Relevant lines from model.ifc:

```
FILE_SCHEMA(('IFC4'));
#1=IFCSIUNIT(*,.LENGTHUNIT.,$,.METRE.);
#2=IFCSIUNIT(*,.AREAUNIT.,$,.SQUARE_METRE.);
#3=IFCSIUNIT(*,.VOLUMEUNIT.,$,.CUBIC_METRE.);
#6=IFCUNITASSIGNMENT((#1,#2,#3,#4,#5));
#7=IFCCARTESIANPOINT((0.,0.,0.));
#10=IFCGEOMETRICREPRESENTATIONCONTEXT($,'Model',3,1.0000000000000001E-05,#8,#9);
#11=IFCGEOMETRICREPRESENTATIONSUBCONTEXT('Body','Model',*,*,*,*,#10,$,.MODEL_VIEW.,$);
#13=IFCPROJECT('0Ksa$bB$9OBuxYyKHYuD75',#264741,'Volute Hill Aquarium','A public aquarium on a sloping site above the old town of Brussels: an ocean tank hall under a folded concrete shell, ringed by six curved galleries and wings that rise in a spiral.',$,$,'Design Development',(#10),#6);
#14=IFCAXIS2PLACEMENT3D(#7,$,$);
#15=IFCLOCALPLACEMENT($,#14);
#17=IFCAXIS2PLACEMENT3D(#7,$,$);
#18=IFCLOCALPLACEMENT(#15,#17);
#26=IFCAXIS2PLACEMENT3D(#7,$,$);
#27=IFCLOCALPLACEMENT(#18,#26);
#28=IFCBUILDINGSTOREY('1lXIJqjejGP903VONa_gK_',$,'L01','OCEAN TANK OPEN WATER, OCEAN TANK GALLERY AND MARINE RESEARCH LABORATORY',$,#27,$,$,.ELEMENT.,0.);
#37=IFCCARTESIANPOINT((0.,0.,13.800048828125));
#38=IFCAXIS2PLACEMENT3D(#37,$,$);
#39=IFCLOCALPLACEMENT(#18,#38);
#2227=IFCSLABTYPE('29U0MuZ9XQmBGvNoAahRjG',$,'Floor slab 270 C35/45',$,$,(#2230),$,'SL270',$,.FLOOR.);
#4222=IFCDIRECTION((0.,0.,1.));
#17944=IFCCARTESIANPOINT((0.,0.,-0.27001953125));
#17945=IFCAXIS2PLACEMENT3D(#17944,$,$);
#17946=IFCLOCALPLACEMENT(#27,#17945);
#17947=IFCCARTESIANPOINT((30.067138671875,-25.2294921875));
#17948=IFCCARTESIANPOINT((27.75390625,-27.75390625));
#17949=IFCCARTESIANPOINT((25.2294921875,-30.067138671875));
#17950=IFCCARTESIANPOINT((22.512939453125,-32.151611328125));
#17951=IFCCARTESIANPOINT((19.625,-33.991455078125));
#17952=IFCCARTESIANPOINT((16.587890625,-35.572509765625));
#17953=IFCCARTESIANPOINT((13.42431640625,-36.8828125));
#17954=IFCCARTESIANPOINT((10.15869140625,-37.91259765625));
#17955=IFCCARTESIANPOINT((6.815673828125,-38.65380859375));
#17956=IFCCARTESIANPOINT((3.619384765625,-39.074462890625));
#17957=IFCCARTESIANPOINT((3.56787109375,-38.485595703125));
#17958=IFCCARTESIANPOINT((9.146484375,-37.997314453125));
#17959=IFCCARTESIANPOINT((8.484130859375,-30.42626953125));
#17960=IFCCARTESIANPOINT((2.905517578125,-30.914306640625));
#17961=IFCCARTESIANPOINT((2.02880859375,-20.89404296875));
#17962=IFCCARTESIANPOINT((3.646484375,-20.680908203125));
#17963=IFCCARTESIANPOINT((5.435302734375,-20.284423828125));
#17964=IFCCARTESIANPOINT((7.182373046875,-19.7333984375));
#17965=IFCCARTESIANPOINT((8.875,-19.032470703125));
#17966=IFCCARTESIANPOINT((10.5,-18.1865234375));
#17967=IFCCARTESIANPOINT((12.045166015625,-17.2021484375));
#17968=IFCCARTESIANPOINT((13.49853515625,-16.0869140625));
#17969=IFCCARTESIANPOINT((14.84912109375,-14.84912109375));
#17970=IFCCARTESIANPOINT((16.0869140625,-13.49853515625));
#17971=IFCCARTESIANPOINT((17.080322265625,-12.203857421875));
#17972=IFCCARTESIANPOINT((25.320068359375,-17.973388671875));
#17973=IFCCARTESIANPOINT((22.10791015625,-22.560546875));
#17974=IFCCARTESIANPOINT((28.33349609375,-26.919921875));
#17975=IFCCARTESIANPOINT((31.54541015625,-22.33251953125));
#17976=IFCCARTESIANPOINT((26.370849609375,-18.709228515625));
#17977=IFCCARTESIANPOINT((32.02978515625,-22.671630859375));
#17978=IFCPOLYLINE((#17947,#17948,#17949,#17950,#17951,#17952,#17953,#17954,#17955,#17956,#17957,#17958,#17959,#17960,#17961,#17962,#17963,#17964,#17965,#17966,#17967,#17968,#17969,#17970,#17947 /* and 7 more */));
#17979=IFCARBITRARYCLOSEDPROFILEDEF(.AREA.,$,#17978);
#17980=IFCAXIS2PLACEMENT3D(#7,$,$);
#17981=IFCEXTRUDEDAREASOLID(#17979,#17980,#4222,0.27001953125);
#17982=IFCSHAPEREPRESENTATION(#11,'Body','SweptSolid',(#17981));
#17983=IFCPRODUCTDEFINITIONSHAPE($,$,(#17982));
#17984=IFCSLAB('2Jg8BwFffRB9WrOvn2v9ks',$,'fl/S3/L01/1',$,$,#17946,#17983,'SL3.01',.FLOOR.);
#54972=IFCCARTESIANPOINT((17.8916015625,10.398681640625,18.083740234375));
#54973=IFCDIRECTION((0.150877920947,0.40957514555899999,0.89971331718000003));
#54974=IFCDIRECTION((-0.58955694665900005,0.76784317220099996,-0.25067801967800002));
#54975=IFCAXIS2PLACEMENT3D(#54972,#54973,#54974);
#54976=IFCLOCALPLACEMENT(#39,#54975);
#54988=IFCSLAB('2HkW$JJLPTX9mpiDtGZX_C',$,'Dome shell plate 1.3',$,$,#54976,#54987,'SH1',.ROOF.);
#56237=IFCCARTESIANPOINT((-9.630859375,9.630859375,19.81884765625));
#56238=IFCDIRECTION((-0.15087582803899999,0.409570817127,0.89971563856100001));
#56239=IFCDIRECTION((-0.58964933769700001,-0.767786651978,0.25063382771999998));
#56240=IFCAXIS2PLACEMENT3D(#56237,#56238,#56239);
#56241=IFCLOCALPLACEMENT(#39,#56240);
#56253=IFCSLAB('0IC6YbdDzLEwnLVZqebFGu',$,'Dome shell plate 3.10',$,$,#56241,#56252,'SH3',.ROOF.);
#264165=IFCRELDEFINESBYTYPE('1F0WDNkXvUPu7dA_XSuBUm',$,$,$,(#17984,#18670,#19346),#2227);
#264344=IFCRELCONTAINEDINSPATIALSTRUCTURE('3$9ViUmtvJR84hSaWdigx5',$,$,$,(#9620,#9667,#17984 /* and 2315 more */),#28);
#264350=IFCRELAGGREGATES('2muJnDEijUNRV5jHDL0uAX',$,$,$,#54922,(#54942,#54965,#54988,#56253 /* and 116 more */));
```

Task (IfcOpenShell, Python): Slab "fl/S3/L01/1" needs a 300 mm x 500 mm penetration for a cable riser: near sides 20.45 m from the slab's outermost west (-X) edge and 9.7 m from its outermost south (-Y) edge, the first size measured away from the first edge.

```python
import numpy as np
import ifcopenshell
import ifcopenshell.api.feature
import ifcopenshell.api.geometry
import ifcopenshell.api.root
import ifcopenshell.geom
import ifcopenshell.util.placement
import ifcopenshell.util.representation
import ifcopenshell.util.shape
import ifcopenshell.util.unit

model = ifcopenshell.open("model.ifc")
unit_scale = ifcopenshell.util.unit.calculate_unit_scale(model)
settings = ifcopenshell.geom.settings()


def volume(element):
    """Net volume in cubic metres, openings subtracted."""
    shape = ifcopenshell.geom.create_shape(settings, element)
    return ifcopenshell.util.shape.get_volume(shape.geometry)


slab = model.by_guid("2Jg8BwFffRB9WrOvn2v9ks")
before = volume(slab)

# Extent in the slab's own axes, in metres. The edges named are its -X and -Y sides.
slab_shape = ifcopenshell.geom.create_shape(settings, slab)
vertices = ifcopenshell.util.shape.get_vertices(slab_shape.geometry)
x_min, y_min, bottom = vertices.min(axis=0)
top = vertices[:, 2].max()

opening = ifcopenshell.api.root.create_entity(model, ifc_class="IfcOpeningElement", name="Cable riser opening", predefined_type="OPENING")
context = ifcopenshell.util.representation.get_context(model, "Model", "Body", "MODEL_VIEW")
width, depth = 0.3, 0.5
outline = [(0.0, 0.0), (width, 0.0), (width, depth), (0.0, depth), (0.0, 0.0)]
# Overshoot both faces by 50 mm so the cut is clean.
shape = ifcopenshell.api.geometry.add_slab_representation(
    model, context=context, depth=top - bottom + 0.1, polyline=outline
)
ifcopenshell.api.geometry.assign_representation(model, product=opening, representation=shape)

matrix = ifcopenshell.util.placement.get_local_placement(slab.ObjectPlacement)
matrix[:, 3] = matrix @ np.append(np.array([x_min + 20.45, y_min + 9.7, bottom - 0.05]) / unit_scale, 1.0)
ifcopenshell.api.geometry.edit_object_placement(model, product=opening, matrix=matrix, is_si=False)
ifcopenshell.api.feature.add_feature(model, feature=opening, element=slab)

after = volume(slab)

print(f"slab volume {before:.3f} -> {after:.3f} m3")

model.write("model_v2.ifc")
```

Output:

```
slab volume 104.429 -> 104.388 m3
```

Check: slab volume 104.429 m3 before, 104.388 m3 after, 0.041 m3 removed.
